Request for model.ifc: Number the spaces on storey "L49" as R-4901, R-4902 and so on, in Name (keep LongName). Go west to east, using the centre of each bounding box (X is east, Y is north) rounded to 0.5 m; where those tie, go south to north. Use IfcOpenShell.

First a look at what the model holds.

```python
import ifcopenshell
import ifcopenshell.util.element
import ifcopenshell.util.placement

model = ifcopenshell.open("model.ifc")
print(model.schema)
storey = next(s for s in model.by_type("IfcBuildingStorey") if s.Name == "L49")
spaces = [e for e in ifcopenshell.util.element.get_decomposition(storey) if e.is_a("IfcSpace")]
for e in sorted(spaces, key=lambda e: e.id()):
    origin = ifcopenshell.util.placement.get_local_placement(e.ObjectPlacement)[:3, 3]
    print(e.id(), e.Name, e.LongName, origin.round(2) + 0.0, sep=" | ")
```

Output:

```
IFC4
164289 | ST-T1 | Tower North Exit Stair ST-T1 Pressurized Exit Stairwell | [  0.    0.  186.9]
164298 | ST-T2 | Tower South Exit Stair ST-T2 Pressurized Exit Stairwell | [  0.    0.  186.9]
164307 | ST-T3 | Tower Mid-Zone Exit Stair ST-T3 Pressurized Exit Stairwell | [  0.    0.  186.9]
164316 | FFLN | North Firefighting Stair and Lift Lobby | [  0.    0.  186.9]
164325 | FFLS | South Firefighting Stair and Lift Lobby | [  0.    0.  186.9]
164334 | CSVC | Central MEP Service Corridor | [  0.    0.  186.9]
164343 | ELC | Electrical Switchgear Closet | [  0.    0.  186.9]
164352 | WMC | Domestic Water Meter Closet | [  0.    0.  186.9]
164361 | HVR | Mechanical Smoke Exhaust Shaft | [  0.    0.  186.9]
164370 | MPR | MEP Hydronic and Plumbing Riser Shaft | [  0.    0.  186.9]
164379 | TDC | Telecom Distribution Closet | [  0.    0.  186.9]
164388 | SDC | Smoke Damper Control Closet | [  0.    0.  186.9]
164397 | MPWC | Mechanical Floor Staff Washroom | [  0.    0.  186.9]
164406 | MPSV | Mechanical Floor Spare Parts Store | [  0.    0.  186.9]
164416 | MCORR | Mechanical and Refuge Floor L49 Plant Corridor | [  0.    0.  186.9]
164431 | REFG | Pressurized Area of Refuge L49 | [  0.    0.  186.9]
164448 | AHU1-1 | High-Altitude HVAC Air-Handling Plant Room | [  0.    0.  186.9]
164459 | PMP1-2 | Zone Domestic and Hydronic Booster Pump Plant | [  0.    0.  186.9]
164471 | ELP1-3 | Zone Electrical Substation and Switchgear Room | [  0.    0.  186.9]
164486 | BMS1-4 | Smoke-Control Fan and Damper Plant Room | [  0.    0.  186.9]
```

```python
import ifcopenshell
import ifcopenshell.geom
import ifcopenshell.util.element
import ifcopenshell.util.shape

model = ifcopenshell.open("model.ifc")
settings = ifcopenshell.geom.settings()
settings.set("use-world-coords", True)


def centre(element):
    shape = ifcopenshell.geom.create_shape(settings, element)
    return ifcopenshell.util.shape.get_bbox_centroid(shape.geometry)


storey = next(s for s in model.by_type("IfcBuildingStorey") if s.Name == "L49")
spaces = [e for e in ifcopenshell.util.element.get_decomposition(storey) if e.is_a("IfcSpace")]

# Insertion points can sit at a corner or the storey origin, so sort by the geometry (in metres).
centres = {e: centre(e) for e in spaces}
spaces.sort(key=lambda e: (round(centres[e][0] / 0.5), centres[e][1]))

for i, e in enumerate(spaces, start=1):
    number = f"R-49{i:02d}"
    e.Name = number
    print(e.id(), number)

model.write("model_edited.ifc")
```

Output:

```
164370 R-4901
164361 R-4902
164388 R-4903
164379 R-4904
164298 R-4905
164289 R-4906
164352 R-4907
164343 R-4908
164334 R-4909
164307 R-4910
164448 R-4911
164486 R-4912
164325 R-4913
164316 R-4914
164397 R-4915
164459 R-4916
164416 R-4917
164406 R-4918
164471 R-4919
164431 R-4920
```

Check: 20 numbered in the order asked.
